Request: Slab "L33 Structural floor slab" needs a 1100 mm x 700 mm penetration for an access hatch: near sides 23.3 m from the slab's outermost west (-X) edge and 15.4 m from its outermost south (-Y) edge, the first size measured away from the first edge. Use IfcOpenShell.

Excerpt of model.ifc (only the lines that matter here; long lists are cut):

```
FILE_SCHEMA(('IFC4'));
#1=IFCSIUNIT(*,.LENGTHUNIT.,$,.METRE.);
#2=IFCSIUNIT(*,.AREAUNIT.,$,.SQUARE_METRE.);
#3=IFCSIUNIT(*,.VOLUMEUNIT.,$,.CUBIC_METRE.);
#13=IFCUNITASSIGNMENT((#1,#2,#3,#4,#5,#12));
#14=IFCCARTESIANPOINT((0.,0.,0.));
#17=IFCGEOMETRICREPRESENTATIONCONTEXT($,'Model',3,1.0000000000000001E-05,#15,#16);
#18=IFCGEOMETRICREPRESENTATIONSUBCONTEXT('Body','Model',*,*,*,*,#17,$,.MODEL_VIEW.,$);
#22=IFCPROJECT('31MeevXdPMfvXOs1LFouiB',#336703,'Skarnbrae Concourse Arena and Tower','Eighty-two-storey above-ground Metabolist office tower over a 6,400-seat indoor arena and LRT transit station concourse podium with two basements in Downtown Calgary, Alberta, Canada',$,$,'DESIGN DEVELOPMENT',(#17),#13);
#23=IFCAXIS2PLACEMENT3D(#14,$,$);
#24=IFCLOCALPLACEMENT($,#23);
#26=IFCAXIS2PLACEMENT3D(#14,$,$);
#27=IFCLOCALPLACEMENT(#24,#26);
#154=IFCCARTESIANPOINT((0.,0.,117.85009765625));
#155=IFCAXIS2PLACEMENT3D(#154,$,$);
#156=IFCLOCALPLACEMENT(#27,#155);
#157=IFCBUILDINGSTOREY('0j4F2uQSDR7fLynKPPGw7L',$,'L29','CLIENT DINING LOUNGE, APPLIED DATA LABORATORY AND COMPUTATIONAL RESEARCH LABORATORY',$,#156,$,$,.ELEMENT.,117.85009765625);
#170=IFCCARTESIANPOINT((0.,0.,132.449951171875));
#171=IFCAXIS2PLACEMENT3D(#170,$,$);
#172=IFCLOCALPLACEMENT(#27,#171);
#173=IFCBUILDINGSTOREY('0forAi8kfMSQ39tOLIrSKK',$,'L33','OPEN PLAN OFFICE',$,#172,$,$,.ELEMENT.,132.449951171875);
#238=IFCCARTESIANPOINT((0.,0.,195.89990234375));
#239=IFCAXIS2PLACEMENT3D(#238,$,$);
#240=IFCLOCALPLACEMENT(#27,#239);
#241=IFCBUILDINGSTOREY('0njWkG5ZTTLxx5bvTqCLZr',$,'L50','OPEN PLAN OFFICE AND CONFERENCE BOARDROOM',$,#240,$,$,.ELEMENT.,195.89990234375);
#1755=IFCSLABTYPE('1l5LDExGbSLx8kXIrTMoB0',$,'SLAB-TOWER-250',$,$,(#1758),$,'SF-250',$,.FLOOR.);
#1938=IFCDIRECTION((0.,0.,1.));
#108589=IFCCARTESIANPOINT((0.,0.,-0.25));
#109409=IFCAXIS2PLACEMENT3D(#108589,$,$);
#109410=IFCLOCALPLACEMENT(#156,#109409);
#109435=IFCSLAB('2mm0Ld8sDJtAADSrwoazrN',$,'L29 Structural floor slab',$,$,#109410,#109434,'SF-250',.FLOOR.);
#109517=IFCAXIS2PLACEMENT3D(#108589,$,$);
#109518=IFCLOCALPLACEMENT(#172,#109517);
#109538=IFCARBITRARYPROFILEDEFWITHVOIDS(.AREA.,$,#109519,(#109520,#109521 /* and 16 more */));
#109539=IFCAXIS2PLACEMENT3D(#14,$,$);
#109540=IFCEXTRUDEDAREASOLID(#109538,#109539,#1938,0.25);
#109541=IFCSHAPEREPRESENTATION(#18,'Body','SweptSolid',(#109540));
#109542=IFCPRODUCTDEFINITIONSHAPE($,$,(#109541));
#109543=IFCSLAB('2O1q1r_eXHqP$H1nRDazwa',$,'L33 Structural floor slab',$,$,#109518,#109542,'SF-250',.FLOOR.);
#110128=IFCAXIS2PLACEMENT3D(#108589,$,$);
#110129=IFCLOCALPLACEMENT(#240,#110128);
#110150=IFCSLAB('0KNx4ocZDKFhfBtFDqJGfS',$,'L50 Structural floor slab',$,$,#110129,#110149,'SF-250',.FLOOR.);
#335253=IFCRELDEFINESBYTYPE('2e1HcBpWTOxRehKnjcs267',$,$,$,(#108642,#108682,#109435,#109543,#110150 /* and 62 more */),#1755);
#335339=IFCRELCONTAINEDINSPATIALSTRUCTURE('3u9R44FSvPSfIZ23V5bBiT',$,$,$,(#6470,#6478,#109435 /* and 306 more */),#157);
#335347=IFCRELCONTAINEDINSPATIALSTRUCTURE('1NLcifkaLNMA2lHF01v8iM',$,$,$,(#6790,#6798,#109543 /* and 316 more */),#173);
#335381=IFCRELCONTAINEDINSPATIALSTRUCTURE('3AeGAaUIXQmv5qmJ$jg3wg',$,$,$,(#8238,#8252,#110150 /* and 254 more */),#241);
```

```python
import numpy as np
import ifcopenshell
import ifcopenshell.api.feature
import ifcopenshell.api.geometry
import ifcopenshell.api.root
import ifcopenshell.geom
import ifcopenshell.util.placement
import ifcopenshell.util.representation
import ifcopenshell.util.shape
import ifcopenshell.util.unit

model = ifcopenshell.open("model.ifc")
unit_scale = ifcopenshell.util.unit.calculate_unit_scale(model)
settings = ifcopenshell.geom.settings()


def volume(element):
    """Net volume in cubic metres, openings subtracted."""
    shape = ifcopenshell.geom.create_shape(settings, element)
    return ifcopenshell.util.shape.get_volume(shape.geometry)


slab = model.by_guid("2O1q1r_eXHqP$H1nRDazwa")
before = volume(slab)

# Extent in the slab's own axes, in metres. The edges named are its -X and -Y sides.
slab_shape = ifcopenshell.geom.create_shape(settings, slab)
vertices = ifcopenshell.util.shape.get_vertices(slab_shape.geometry)
x_min, y_min, bottom = vertices.min(axis=0)
top = vertices[:, 2].max()

opening = ifcopenshell.api.root.create_entity(model, ifc_class="IfcOpeningElement", name="Access hatch opening", predefined_type="OPENING")
context = ifcopenshell.util.representation.get_context(model, "Model", "Body", "MODEL_VIEW")
width, depth = 1.1, 0.7
outline = [(0.0, 0.0), (width, 0.0), (width, depth), (0.0, depth), (0.0, 0.0)]
# Overshoot both faces by 50 mm so the cut is clean.
shape = ifcopenshell.api.geometry.add_slab_representation(
    model, context=context, depth=top - bottom + 0.1, polyline=outline
)
ifcopenshell.api.geometry.assign_representation(model, product=opening, representation=shape)

matrix = ifcopenshell.util.placement.get_local_placement(slab.ObjectPlacement)
matrix[:, 3] = matrix @ np.append(np.array([x_min + 23.3, y_min + 15.4, bottom - 0.05]) / unit_scale, 1.0)
ifcopenshell.api.geometry.edit_object_placement(model, product=opening, matrix=matrix, is_si=False)
ifcopenshell.api.feature.add_feature(model, feature=opening, element=slab)

after = volume(slab)

print(f"slab volume {before:.3f} -> {after:.3f} m3")

model.write("model_updated.ifc")
```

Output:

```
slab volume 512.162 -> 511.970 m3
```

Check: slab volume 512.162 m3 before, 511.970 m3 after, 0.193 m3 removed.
